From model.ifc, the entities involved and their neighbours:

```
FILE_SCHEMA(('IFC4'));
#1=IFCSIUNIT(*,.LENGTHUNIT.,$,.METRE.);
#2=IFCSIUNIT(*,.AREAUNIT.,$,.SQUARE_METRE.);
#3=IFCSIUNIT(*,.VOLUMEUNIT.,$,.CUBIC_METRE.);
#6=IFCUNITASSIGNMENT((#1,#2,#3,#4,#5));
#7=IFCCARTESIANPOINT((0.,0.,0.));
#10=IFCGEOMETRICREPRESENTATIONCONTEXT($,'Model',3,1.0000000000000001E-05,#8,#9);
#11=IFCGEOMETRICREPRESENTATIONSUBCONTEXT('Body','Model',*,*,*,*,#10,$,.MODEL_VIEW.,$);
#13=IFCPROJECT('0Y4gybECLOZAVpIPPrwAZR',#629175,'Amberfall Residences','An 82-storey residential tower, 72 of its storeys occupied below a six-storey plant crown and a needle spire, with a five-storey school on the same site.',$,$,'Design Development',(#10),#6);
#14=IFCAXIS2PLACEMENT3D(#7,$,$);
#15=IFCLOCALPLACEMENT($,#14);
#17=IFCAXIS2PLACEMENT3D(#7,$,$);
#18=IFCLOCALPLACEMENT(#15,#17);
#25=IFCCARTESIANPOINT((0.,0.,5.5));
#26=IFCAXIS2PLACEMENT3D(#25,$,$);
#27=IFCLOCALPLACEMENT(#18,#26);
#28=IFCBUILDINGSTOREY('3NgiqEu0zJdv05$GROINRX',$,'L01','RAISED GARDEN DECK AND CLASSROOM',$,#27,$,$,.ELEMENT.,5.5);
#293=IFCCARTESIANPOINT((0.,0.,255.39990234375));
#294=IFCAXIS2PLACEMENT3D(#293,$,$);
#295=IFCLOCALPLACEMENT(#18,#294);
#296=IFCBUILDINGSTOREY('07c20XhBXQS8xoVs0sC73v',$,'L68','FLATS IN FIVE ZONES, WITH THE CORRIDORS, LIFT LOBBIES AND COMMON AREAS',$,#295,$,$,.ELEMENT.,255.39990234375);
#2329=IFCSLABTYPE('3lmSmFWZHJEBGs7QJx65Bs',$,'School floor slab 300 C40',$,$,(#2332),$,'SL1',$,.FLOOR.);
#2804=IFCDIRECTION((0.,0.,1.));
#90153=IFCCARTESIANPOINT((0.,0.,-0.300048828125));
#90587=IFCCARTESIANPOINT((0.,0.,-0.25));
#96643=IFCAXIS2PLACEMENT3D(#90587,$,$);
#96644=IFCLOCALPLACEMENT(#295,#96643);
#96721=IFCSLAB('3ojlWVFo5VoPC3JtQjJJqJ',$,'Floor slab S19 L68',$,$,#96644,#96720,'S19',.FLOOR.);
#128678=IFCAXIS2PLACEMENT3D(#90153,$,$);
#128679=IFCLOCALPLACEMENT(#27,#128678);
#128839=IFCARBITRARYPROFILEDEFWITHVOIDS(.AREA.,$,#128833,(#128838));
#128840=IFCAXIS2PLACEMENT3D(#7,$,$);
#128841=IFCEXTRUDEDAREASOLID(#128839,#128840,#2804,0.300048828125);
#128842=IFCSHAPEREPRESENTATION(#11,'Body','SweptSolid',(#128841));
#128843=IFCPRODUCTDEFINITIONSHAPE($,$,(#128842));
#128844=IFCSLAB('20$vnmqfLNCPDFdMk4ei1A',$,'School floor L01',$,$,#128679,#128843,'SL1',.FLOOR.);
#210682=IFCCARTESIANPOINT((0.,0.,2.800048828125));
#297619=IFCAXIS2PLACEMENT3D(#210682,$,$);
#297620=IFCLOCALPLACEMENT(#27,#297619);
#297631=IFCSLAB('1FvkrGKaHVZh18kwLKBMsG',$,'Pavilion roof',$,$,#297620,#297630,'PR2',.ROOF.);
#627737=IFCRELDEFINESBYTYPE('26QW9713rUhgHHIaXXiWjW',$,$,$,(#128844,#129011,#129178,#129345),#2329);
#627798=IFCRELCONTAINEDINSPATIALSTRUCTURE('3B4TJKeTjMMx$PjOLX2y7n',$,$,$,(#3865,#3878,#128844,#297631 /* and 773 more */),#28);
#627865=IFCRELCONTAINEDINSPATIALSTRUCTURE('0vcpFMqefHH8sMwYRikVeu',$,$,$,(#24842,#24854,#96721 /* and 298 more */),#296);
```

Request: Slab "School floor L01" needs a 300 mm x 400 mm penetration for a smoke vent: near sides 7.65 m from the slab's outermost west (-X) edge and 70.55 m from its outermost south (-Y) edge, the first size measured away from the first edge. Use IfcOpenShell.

```python
import numpy as np
import ifcopenshell
import ifcopenshell.api.feature
import ifcopenshell.api.geometry
import ifcopenshell.api.root
import ifcopenshell.geom
import ifcopenshell.util.placement
import ifcopenshell.util.representation
import ifcopenshell.util.shape
import ifcopenshell.util.unit

model = ifcopenshell.open("model.ifc")
unit_scale = ifcopenshell.util.unit.calculate_unit_scale(model)
settings = ifcopenshell.geom.settings()


def volume(element):
    """Net volume in cubic metres, openings subtracted."""
    shape = ifcopenshell.geom.create_shape(settings, element)
    return ifcopenshell.util.shape.get_volume(shape.geometry)


slab = model.by_guid("20$vnmqfLNCPDFdMk4ei1A")
before = volume(slab)

# Extent in the slab's own axes, in metres. The edges named are its -X and -Y sides.
slab_shape = ifcopenshell.geom.create_shape(settings, slab)
vertices = ifcopenshell.util.shape.get_vertices(slab_shape.geometry)
x_min, y_min, bottom = vertices.min(axis=0)
top = vertices[:, 2].max()

opening = ifcopenshell.api.root.create_entity(model, ifc_class="IfcOpeningElement", name="Smoke vent opening", predefined_type="OPENING")
context = ifcopenshell.util.representation.get_context(model, "Model", "Body", "MODEL_VIEW")
width, depth = 0.3, 0.4
outline = [(0.0, 0.0), (width, 0.0), (width, depth), (0.0, depth), (0.0, 0.0)]
# Overshoot both faces by 50 mm so the cut is clean.
shape = ifcopenshell.api.geometry.add_slab_representation(
    model, context=context, depth=top - bottom + 0.1, polyline=outline
)
ifcopenshell.api.geometry.assign_representation(model, product=opening, representation=shape)

matrix = ifcopenshell.util.placement.get_local_placement(slab.ObjectPlacement)
matrix[:, 3] = matrix @ np.append(np.array([x_min + 7.65, y_min + 70.55, bottom - 0.05]) / unit_scale, 1.0)
ifcopenshell.api.geometry.edit_object_placement(model, product=opening, matrix=matrix, is_si=False)
ifcopenshell.api.feature.add_feature(model, feature=opening, element=slab)

after = volume(slab)

print(f"slab volume {before:.3f} -> {after:.3f} m3")

model.write("model_updated.ifc")
```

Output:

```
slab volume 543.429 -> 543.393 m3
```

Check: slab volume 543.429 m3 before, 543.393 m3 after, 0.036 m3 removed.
